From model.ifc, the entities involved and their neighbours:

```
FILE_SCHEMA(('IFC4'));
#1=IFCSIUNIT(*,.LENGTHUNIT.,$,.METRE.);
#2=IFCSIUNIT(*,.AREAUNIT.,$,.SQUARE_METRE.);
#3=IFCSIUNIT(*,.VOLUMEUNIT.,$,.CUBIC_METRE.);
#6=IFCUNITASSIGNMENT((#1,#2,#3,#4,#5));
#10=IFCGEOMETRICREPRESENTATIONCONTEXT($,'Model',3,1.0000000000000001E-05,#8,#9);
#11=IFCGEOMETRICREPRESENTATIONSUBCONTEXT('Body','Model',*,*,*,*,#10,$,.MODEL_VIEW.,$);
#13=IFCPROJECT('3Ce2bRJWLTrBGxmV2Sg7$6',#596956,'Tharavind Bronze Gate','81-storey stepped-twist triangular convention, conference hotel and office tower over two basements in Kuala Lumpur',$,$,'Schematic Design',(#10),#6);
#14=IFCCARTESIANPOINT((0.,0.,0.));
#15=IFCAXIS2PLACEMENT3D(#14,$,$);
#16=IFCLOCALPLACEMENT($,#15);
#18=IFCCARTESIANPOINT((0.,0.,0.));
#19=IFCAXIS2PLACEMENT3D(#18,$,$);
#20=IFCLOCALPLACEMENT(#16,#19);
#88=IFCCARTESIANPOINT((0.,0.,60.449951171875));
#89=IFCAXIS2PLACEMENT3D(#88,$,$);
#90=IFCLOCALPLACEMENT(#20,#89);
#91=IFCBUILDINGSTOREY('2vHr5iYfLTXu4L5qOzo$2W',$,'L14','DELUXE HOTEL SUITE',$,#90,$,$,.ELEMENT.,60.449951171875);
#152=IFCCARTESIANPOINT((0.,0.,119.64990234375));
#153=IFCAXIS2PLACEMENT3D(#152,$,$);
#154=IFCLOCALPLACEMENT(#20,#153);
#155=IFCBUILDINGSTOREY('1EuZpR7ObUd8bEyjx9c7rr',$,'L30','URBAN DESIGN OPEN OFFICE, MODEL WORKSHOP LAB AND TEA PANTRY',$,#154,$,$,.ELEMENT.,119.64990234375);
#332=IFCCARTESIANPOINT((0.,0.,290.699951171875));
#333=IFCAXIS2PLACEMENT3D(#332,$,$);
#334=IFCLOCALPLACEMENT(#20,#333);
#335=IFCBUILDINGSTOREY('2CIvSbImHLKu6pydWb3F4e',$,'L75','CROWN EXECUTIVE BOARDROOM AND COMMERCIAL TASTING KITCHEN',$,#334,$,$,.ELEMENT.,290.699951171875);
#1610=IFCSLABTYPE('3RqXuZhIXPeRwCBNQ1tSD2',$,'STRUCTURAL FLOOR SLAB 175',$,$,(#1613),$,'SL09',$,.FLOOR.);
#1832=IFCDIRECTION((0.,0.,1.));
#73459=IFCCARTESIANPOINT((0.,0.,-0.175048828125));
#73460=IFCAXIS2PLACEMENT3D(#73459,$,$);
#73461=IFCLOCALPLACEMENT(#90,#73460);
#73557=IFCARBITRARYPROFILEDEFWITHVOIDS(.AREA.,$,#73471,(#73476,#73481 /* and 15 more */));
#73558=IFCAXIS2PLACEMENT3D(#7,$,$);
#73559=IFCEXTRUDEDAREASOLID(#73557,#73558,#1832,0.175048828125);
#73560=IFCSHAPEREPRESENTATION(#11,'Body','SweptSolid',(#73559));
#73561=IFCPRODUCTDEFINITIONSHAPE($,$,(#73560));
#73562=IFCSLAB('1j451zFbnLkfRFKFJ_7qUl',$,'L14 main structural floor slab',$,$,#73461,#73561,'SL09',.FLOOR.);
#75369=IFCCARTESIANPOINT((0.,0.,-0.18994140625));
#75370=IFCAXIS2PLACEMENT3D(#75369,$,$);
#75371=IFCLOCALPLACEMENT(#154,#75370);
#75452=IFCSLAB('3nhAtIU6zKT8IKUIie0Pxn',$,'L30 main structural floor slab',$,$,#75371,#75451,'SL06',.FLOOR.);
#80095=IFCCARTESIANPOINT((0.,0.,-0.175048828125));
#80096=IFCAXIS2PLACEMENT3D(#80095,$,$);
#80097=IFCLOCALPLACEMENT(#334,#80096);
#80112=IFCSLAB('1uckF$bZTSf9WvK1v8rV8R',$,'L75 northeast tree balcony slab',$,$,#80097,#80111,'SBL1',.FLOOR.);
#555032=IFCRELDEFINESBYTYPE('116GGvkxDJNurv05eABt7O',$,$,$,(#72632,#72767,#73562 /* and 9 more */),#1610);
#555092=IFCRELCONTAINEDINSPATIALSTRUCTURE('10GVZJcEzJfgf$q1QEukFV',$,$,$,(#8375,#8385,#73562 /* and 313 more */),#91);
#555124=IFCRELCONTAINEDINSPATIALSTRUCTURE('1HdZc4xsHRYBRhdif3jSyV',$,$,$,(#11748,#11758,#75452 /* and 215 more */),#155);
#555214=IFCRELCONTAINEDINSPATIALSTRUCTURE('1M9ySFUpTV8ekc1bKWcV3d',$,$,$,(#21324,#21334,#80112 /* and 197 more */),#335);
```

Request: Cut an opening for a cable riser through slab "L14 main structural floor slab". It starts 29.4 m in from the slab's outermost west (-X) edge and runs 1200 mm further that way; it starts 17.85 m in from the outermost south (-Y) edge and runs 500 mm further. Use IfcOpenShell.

```python
import numpy as np
import ifcopenshell
import ifcopenshell.api.feature
import ifcopenshell.api.geometry
import ifcopenshell.api.root
import ifcopenshell.geom
import ifcopenshell.util.placement
import ifcopenshell.util.representation
import ifcopenshell.util.shape
import ifcopenshell.util.unit

model = ifcopenshell.open("model.ifc")
unit_scale = ifcopenshell.util.unit.calculate_unit_scale(model)
settings = ifcopenshell.geom.settings()


def volume(element):
    """Net volume in cubic metres, openings subtracted."""
    shape = ifcopenshell.geom.create_shape(settings, element)
    return ifcopenshell.util.shape.get_volume(shape.geometry)


slab = model.by_id(73562)
before = volume(slab)

# Extent in the slab's own axes, in metres. The edges named are its -X and -Y sides.
slab_shape = ifcopenshell.geom.create_shape(settings, slab)
vertices = ifcopenshell.util.shape.get_vertices(slab_shape.geometry)
x_min, y_min, bottom = vertices.min(axis=0)
top = vertices[:, 2].max()

opening = ifcopenshell.api.root.create_entity(model, ifc_class="IfcOpeningElement", name="Cable riser opening", predefined_type="OPENING")
context = ifcopenshell.util.representation.get_context(model, "Model", "Body", "MODEL_VIEW")
width, depth = 1.2, 0.5
outline = [(0.0, 0.0), (width, 0.0), (width, depth), (0.0, depth), (0.0, 0.0)]
# Overshoot both faces by 50 mm so the cut is clean.
shape = ifcopenshell.api.geometry.add_slab_representation(
    model, context=context, depth=top - bottom + 0.1, polyline=outline
)
ifcopenshell.api.geometry.assign_representation(model, product=opening, representation=shape)

matrix = ifcopenshell.util.placement.get_local_placement(slab.ObjectPlacement)
matrix[:, 3] = matrix @ np.append(np.array([x_min + 29.4, y_min + 17.85, bottom - 0.05]) / unit_scale, 1.0)
ifcopenshell.api.geometry.edit_object_placement(model, product=opening, matrix=matrix, is_si=False)
ifcopenshell.api.feature.add_feature(model, feature=opening, element=slab)

after = volume(slab)

print(f"slab volume {before:.3f} -> {after:.3f} m3")

model.write("model_updated.ifc")
```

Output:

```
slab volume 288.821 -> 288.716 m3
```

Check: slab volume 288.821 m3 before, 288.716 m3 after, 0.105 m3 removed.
